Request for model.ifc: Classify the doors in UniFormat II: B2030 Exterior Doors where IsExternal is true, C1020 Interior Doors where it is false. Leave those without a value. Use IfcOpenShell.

First a look at what the model holds.

```python
import ifcopenshell
import ifcopenshell.util.element

model = ifcopenshell.open("model.ifc")
print(model.schema)
print("classifications:", [c.Name for c in model.by_type("IfcClassification")])
values = [ifcopenshell.util.element.get_pset(e, "Pset_DoorCommon", "IsExternal") for e in model.by_type("IfcDoor")]
for value in (True, False, None):
    print("IsExternal", value, values.count(value))
```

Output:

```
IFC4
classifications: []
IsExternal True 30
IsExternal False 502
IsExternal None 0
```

```python
import ifcopenshell
import ifcopenshell.api.classification
import ifcopenshell.util.element

model = ifcopenshell.open("model.ifc")

system = ifcopenshell.api.classification.add_classification(model, classification="UniFormat II")

doors = model.by_type("IfcDoor")
external = {e: ifcopenshell.util.element.get_pset(e, "Pset_DoorCommon", "IsExternal") for e in doors}
for flag, code, name in ((True, "B2030", "Exterior Doors"), (False, "C1020", "Interior Doors")):
    products = [e for e in doors if external[e] is flag]
    ifcopenshell.api.classification.add_reference(
        model, products=products, classification=system, identification=code, name=name
    )
    print(code, len(products))

model.write("model_updated.ifc")
```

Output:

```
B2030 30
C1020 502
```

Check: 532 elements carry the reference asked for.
